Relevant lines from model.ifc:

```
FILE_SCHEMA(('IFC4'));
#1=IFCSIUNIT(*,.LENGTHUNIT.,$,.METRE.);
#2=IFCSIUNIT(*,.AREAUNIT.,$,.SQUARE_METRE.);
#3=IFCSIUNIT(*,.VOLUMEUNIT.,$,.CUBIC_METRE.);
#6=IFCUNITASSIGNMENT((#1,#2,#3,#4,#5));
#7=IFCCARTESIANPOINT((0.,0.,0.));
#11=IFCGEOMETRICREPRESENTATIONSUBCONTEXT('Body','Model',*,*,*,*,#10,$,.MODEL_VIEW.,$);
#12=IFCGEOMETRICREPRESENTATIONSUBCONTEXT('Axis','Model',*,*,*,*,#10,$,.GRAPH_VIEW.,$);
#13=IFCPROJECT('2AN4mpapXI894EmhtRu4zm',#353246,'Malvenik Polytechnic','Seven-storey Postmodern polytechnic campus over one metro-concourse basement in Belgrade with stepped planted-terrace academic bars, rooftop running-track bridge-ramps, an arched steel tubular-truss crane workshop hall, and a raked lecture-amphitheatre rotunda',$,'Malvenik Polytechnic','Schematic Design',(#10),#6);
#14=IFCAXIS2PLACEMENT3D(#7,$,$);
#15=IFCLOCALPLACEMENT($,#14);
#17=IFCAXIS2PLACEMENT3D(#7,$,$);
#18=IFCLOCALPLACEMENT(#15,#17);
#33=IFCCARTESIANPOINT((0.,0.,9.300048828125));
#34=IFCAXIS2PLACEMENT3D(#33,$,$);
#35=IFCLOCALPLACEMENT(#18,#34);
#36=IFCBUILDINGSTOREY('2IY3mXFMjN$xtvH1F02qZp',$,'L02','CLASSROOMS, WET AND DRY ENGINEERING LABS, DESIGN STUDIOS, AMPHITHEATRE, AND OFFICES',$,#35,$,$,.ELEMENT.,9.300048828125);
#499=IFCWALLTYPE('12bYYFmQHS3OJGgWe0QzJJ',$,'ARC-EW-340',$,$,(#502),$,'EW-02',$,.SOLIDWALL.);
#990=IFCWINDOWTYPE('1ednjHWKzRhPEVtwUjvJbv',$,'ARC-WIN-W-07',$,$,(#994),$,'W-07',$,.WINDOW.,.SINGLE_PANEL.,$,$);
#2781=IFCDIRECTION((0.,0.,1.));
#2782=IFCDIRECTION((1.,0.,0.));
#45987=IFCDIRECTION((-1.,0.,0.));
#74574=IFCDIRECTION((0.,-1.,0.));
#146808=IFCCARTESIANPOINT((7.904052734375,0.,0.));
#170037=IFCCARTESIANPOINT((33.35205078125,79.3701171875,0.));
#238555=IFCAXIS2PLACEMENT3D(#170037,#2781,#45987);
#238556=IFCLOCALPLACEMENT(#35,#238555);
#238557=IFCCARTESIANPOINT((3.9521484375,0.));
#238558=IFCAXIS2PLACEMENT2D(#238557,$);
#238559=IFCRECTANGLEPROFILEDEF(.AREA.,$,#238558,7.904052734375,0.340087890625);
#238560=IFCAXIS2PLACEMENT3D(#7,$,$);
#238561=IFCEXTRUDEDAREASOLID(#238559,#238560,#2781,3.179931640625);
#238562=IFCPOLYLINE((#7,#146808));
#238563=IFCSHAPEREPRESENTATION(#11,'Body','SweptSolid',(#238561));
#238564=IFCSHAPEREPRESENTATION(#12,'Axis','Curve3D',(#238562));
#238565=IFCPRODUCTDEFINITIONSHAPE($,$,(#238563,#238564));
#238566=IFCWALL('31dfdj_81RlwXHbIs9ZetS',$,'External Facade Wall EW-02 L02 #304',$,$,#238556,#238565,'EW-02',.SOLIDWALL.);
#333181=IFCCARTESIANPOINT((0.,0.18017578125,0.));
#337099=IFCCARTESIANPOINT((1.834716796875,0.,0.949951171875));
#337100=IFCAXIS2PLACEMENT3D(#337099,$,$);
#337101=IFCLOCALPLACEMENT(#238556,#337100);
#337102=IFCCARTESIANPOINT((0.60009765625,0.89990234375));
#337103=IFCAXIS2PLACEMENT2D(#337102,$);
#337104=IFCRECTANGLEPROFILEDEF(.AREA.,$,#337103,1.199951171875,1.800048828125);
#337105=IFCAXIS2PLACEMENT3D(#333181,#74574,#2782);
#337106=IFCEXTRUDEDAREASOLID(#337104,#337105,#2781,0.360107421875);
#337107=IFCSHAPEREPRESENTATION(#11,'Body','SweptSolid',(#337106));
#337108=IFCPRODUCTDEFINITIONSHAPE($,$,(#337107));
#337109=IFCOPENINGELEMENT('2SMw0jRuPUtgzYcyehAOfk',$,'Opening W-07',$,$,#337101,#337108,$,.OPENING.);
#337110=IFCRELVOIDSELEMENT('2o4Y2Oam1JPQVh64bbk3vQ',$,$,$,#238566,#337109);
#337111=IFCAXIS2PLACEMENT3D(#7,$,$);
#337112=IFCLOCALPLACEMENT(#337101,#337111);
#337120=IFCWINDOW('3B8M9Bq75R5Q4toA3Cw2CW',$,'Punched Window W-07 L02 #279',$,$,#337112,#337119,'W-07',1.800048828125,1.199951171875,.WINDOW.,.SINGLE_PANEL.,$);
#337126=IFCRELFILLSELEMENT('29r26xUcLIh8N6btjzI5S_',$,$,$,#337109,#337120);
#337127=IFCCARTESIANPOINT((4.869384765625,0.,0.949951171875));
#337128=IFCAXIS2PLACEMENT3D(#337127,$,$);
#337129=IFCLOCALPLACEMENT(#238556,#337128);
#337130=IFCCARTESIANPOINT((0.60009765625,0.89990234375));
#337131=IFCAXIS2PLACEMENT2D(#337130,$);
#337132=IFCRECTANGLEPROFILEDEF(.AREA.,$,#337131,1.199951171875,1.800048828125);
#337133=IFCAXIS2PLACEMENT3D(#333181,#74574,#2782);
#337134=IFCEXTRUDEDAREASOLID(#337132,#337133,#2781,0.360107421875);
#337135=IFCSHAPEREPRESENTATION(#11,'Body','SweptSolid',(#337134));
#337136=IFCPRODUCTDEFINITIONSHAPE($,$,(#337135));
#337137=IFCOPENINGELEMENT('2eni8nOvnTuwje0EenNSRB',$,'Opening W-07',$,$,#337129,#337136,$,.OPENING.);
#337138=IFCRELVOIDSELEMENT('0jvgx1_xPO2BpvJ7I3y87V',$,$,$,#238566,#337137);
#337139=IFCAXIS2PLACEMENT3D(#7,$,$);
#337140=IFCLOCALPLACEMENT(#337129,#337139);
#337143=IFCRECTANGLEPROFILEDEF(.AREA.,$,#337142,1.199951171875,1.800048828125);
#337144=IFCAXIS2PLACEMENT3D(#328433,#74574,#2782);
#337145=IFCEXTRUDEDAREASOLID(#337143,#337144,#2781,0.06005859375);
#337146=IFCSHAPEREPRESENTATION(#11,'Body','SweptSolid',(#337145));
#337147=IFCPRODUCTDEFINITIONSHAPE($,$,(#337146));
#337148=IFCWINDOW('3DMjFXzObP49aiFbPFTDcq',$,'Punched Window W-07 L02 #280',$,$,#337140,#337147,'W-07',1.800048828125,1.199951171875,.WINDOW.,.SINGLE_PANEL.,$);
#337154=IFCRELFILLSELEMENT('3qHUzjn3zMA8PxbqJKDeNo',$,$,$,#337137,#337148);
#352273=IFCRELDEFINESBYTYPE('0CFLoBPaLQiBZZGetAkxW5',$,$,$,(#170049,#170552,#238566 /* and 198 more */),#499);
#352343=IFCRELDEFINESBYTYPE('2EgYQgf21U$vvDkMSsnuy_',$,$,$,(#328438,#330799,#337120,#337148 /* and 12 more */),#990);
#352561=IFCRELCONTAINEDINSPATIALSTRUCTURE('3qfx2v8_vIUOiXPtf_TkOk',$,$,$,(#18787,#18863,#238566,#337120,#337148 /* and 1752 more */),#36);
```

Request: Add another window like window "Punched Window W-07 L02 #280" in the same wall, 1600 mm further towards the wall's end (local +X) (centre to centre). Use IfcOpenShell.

```python
import ifcopenshell
import ifcopenshell.api.feature
import ifcopenshell.api.geometry
import ifcopenshell.api.root
import ifcopenshell.geom
import ifcopenshell.util.element
import ifcopenshell.util.placement
import ifcopenshell.util.shape
import ifcopenshell.util.unit

model = ifcopenshell.open("model.ifc")
unit_scale = ifcopenshell.util.unit.calculate_unit_scale(model)
settings = ifcopenshell.geom.settings()


def volume(element):
    """Net volume in cubic metres, openings subtracted."""
    shape = ifcopenshell.geom.create_shape(settings, element)
    return ifcopenshell.util.shape.get_volume(shape.geometry)


window = model.by_guid("3DMjFXzObP49aiFbPFTDcq")
opening = window.FillsVoids[0].RelatingOpeningElement
wall = opening.VoidsElements[0].RelatingBuildingElement
before = volume(wall)
shift = ifcopenshell.util.placement.get_local_placement(wall.ObjectPlacement)[:3, 0] * 1.6 / unit_scale

# copy_class copies the void relationship, type, container and properties, but no geometry.
new_opening = ifcopenshell.api.root.copy_class(model, product=opening)
new_opening.Representation = ifcopenshell.util.element.copy_deep(
    model, opening.Representation, exclude=["IfcGeometricRepresentationContext", "IfcRepresentationMap"]
)
new_window = ifcopenshell.api.root.copy_class(model, product=window)
new_window.Representation = ifcopenshell.util.element.copy_deep(
    model, window.Representation, exclude=["IfcGeometricRepresentationContext", "IfcRepresentationMap"]
)
new_window.Tag = None
ifcopenshell.api.feature.add_filling(model, opening=new_opening, element=new_window)

for old, new in ((opening, new_opening), (window, new_window)):
    matrix = ifcopenshell.util.placement.get_local_placement(old.ObjectPlacement)
    matrix[:3, 3] += shift
    ifcopenshell.api.geometry.edit_object_placement(model, product=new, matrix=matrix, is_si=False)

after = volume(wall)

print(f"wall volume {before:.3f} -> {after:.3f} m3")

model.write("model_v2.ifc")
```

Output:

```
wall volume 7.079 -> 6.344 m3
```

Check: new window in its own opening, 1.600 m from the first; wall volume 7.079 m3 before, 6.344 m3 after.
